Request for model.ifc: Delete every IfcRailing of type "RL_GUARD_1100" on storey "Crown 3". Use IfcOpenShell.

First a look at what the model holds.

```python
import ifcopenshell
import ifcopenshell.util.element

model = ifcopenshell.open("model.ifc")
print(model.schema)
storey = next(s for s in model.by_type("IfcBuildingStorey") if s.Name == "Crown 3")
railings = [e for e in ifcopenshell.util.element.get_decomposition(storey) if e.is_a("IfcRailing")]
seen = {}
for e in railings:
    element_type = ifcopenshell.util.element.get_type(e)
    name = element_type.Name if element_type not in (None, e) else None
    seen[name] = seen.get(name, 0) + 1
for name, count in sorted(seen.items(), key=str):
    print(count, "x", name)
```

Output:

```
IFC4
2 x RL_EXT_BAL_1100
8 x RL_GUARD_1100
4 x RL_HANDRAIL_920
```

```python
import ifcopenshell
import ifcopenshell.api.root
import ifcopenshell.util.element

model = ifcopenshell.open("model.ifc")

storey = next(s for s in model.by_type("IfcBuildingStorey") if s.Name == "Crown 3")
railings = [e for e in ifcopenshell.util.element.get_decomposition(storey) if e.is_a("IfcRailing")]
targets = [e for e in railings if (t := ifcopenshell.util.element.get_type(e)) not in (None, e) and t.Name == "RL_GUARD_1100"]

for e in targets:
    ifcopenshell.api.root.remove_product(model, product=e)
print(len(targets), "removed")

model.write("model_updated.ifc")
```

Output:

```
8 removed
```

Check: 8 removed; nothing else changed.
